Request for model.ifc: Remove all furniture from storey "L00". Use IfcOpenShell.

First a look at what the model holds.

```python
import ifcopenshell
import ifcopenshell.util.element

model = ifcopenshell.open("model.ifc")
print(model.schema)
storey = next(s for s in model.by_type("IfcBuildingStorey") if s.Name == "L00")
furniture = [e for e in ifcopenshell.util.element.get_decomposition(storey) if e.is_a("IfcFurnishingElement")]
seen = {}
for e in furniture:
    element_type = ifcopenshell.util.element.get_type(e)
    name = element_type.Name if element_type not in (None, e) else None
    seen[name] = seen.get(name, 0) + 1
for name, count in sorted(seen.items(), key=str):
    print(count, "x", name)
```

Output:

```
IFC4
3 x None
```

```python
import ifcopenshell
import ifcopenshell.api.root
import ifcopenshell.util.element

model = ifcopenshell.open("model.ifc")

storey = next(s for s in model.by_type("IfcBuildingStorey") if s.Name == "L00")
furniture = [e for e in ifcopenshell.util.element.get_decomposition(storey) if e.is_a("IfcFurnishingElement")]

for e in furniture:
    ifcopenshell.api.root.remove_product(model, product=e)
print(len(furniture), "removed")

model.write("model_edited.ifc")
```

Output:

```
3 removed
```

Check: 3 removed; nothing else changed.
